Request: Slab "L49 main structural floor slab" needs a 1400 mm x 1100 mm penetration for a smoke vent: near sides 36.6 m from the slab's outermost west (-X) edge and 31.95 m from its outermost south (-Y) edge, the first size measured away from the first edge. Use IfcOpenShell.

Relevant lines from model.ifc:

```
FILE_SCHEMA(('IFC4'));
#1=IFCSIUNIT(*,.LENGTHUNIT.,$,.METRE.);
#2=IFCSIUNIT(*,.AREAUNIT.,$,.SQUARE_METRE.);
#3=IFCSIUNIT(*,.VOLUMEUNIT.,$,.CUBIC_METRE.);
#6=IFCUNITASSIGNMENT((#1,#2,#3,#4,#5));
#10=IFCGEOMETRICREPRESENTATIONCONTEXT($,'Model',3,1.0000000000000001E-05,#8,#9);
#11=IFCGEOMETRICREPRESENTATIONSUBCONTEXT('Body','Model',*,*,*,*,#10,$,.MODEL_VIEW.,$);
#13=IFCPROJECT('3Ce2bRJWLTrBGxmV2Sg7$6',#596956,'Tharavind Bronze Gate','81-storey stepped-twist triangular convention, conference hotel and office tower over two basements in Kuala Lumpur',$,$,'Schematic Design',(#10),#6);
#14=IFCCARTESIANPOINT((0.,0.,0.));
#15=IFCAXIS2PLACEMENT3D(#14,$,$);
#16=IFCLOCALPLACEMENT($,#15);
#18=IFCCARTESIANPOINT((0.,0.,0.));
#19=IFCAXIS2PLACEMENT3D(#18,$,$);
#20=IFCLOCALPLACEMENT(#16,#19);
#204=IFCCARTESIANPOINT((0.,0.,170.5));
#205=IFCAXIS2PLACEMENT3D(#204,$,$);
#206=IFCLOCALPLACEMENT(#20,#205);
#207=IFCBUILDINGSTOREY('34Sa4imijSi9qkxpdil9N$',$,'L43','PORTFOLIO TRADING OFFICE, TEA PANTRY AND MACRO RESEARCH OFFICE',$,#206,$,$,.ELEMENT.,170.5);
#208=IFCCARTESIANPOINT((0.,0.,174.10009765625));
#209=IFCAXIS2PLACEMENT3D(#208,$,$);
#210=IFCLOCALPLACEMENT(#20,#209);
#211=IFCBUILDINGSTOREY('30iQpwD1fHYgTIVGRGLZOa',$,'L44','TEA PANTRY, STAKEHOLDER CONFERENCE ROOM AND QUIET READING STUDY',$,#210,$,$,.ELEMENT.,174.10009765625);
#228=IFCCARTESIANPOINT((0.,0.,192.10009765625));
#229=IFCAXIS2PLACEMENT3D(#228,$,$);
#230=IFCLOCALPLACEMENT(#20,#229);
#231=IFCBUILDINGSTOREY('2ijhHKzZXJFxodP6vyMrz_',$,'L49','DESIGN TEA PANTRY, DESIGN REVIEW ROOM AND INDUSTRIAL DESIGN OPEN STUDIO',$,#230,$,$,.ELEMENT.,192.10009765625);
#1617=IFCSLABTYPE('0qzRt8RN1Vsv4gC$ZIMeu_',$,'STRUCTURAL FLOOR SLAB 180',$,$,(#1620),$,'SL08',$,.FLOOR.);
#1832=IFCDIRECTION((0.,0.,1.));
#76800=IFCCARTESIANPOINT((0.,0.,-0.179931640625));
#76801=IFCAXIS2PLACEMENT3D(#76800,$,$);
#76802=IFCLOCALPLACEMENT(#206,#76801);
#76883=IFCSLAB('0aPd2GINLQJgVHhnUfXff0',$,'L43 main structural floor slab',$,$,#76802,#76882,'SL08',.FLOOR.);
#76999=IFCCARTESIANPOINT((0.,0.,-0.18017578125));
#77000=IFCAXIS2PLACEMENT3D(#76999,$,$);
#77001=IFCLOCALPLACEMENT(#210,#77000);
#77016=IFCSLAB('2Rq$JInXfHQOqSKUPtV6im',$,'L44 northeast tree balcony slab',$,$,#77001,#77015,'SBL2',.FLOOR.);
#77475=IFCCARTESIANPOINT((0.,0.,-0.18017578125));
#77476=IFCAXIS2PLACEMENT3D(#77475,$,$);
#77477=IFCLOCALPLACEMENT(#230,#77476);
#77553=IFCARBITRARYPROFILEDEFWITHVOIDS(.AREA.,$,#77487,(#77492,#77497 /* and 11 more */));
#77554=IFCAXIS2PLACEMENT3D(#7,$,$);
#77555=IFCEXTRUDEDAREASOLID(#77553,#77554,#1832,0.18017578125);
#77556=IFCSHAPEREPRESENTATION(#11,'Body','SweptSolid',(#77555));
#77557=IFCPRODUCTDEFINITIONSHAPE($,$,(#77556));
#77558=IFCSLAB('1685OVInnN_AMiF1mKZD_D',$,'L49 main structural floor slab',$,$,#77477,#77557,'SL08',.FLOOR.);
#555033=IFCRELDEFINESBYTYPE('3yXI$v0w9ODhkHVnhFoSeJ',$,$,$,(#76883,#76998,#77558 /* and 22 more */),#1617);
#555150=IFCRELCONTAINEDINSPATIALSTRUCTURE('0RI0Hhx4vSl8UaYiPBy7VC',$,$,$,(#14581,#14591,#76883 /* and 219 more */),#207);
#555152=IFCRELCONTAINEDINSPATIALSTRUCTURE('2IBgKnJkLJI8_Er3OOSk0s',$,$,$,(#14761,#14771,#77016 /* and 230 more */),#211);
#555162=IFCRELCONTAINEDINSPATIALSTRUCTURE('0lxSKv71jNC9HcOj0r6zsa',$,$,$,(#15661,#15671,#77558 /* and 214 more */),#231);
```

```python
import numpy as np
import ifcopenshell
import ifcopenshell.api.feature
import ifcopenshell.api.geometry
import ifcopenshell.api.root
import ifcopenshell.geom
import ifcopenshell.util.placement
import ifcopenshell.util.representation
import ifcopenshell.util.shape
import ifcopenshell.util.unit

model = ifcopenshell.open("model.ifc")
unit_scale = ifcopenshell.util.unit.calculate_unit_scale(model)
settings = ifcopenshell.geom.settings()


def volume(element):
    """Net volume in cubic metres, openings subtracted."""
    shape = ifcopenshell.geom.create_shape(settings, element)
    return ifcopenshell.util.shape.get_volume(shape.geometry)


slab = model.by_guid("1685OVInnN_AMiF1mKZD_D")
before = volume(slab)

# Extent in the slab's own axes, in metres. The edges named are its -X and -Y sides.
slab_shape = ifcopenshell.geom.create_shape(settings, slab)
vertices = ifcopenshell.util.shape.get_vertices(slab_shape.geometry)
x_min, y_min, bottom = vertices.min(axis=0)
top = vertices[:, 2].max()

opening = ifcopenshell.api.root.create_entity(model, ifc_class="IfcOpeningElement", name="Smoke vent opening", predefined_type="OPENING")
context = ifcopenshell.util.representation.get_context(model, "Model", "Body", "MODEL_VIEW")
width, depth = 1.4, 1.1
outline = [(0.0, 0.0), (width, 0.0), (width, depth), (0.0, depth), (0.0, 0.0)]
# Overshoot both faces by 50 mm so the cut is clean.
shape = ifcopenshell.api.geometry.add_slab_representation(
    model, context=context, depth=top - bottom + 0.1, polyline=outline
)
ifcopenshell.api.geometry.assign_representation(model, product=opening, representation=shape)

matrix = ifcopenshell.util.placement.get_local_placement(slab.ObjectPlacement)
matrix[:, 3] = matrix @ np.append(np.array([x_min + 36.6, y_min + 31.95, bottom - 0.05]) / unit_scale, 1.0)
ifcopenshell.api.geometry.edit_object_placement(model, product=opening, matrix=matrix, is_si=False)
ifcopenshell.api.feature.add_feature(model, feature=opening, element=slab)

after = volume(slab)

print(f"slab volume {before:.3f} -> {after:.3f} m3")

model.write("model_rev.ifc")
```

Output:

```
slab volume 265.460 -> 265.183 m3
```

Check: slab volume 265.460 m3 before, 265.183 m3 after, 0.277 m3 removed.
